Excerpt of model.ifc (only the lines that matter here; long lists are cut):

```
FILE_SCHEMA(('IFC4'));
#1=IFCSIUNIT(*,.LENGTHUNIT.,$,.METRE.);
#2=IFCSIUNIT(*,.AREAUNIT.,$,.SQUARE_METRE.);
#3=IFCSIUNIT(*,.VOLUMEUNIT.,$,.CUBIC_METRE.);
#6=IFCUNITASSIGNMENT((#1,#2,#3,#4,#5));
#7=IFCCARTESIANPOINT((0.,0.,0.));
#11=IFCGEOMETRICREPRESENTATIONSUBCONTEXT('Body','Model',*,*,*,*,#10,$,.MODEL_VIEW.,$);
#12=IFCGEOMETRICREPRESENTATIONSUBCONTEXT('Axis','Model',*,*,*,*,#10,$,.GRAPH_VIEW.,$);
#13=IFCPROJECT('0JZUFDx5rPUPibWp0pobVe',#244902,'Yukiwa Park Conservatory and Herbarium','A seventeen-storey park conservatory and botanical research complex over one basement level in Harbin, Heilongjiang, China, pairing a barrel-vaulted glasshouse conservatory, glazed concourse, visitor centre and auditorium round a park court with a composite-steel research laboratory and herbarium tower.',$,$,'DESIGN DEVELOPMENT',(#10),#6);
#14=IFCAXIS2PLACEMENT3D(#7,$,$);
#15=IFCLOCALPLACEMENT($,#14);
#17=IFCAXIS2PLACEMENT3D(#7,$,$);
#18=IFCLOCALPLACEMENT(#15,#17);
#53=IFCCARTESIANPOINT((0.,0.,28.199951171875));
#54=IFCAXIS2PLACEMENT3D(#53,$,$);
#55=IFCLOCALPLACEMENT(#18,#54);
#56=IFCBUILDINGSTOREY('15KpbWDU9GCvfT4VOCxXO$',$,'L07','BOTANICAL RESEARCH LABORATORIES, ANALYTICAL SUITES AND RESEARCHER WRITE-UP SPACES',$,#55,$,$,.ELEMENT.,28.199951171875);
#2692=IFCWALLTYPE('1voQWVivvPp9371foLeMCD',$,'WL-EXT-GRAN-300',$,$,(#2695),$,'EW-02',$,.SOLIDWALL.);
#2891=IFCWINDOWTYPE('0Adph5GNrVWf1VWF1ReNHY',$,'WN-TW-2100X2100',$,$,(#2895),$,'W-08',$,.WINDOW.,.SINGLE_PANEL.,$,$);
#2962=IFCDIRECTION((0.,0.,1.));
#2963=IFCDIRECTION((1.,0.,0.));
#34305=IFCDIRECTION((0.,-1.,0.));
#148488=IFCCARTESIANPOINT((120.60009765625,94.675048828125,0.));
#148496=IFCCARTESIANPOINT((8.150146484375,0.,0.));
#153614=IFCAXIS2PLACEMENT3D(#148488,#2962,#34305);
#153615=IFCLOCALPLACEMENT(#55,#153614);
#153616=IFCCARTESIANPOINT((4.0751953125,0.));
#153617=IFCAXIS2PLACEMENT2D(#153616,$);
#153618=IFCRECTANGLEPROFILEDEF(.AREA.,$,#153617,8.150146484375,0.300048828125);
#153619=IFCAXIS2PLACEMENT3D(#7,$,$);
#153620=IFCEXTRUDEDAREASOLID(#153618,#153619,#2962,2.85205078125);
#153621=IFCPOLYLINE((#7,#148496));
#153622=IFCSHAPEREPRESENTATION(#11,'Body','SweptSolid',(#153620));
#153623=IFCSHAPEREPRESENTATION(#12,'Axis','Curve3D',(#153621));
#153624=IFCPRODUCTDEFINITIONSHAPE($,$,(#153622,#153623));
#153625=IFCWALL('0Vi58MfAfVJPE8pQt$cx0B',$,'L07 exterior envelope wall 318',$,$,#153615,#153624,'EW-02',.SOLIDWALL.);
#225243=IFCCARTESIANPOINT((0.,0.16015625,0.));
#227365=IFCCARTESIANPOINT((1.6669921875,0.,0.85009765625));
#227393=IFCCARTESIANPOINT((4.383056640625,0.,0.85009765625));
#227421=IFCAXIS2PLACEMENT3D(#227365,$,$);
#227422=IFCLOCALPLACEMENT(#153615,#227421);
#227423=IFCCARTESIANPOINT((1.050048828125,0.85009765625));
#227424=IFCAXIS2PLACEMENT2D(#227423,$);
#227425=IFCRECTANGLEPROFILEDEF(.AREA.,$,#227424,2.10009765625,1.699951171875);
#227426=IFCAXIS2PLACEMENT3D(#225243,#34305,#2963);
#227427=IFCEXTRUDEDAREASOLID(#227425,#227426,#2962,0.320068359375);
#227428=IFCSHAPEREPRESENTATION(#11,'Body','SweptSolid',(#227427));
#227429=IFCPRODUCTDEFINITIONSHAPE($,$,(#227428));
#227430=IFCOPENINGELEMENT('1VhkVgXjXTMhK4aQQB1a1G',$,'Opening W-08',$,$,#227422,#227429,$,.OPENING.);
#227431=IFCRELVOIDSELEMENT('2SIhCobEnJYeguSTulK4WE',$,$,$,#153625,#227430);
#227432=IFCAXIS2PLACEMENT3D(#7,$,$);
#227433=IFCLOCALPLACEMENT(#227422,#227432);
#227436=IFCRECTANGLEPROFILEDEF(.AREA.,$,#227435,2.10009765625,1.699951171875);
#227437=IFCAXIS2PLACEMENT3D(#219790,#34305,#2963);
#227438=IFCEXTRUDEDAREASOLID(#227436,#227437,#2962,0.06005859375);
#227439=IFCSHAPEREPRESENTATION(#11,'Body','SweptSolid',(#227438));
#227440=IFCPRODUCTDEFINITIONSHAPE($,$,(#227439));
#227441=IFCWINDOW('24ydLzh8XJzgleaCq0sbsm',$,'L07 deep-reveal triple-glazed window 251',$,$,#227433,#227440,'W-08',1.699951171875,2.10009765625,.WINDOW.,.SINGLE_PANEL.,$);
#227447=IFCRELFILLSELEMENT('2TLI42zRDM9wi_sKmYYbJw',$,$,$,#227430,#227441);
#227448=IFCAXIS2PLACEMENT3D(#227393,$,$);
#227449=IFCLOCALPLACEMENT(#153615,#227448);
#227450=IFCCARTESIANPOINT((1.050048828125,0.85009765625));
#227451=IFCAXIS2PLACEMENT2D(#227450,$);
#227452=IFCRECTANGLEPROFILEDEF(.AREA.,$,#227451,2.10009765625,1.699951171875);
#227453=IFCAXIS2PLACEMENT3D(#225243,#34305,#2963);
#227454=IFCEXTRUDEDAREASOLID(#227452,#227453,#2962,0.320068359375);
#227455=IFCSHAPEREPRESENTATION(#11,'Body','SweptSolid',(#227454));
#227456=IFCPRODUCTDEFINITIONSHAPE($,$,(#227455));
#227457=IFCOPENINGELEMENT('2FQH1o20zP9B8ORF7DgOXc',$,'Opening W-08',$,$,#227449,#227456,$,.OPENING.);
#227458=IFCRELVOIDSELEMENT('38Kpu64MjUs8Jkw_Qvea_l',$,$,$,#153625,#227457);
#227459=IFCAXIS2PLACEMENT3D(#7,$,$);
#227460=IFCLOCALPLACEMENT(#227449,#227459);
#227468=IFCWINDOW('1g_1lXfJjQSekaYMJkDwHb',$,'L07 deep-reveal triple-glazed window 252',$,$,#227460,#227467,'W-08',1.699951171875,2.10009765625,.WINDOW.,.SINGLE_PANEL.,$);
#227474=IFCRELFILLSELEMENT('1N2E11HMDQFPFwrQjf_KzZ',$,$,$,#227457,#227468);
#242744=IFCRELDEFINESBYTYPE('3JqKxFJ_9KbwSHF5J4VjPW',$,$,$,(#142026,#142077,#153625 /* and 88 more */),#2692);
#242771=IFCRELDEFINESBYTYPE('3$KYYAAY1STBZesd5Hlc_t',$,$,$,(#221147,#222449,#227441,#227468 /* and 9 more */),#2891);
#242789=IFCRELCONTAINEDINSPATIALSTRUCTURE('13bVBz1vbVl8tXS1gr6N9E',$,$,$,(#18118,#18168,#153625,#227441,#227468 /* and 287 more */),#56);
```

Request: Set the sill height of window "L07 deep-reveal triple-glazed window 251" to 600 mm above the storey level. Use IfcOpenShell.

```python
import numpy as np
import ifcopenshell
import ifcopenshell.api.geometry
import ifcopenshell.geom
import ifcopenshell.util.element
import ifcopenshell.util.placement
import ifcopenshell.util.shape
import ifcopenshell.util.unit

model = ifcopenshell.open("model.ifc")
unit_scale = ifcopenshell.util.unit.calculate_unit_scale(model)

window = model.by_guid("24ydLzh8XJzgleaCq0sbsm")
opening = window.FillsVoids[0].RelatingOpeningElement
storey = ifcopenshell.util.element.get_container(window, ifc_class="IfcBuildingStorey")
level = ifcopenshell.util.placement.get_local_placement(storey.ObjectPlacement)[2, 3]

# The opening's origin need not be at the sill, so measure its lowest point.
shape = ifcopenshell.geom.create_shape(ifcopenshell.geom.settings(), opening)
bottom = ifcopenshell.util.shape.get_shape_bottom_elevation(shape, shape.geometry) / unit_scale
dz = level + 0.6 - bottom

shift = np.array([0.0, 0.0, dz])
# The window is placed relative to its opening, so it follows when the opening moves.
matrix = ifcopenshell.util.placement.get_local_placement(opening.ObjectPlacement)
matrix[:3, 3] += shift
ifcopenshell.api.geometry.edit_object_placement(
    model, product=opening, matrix=matrix, is_si=False, should_transform_children=True
)

print(f"moved by {dz * unit_scale:+.3f} m")

model.write("model_rev.ifc")
```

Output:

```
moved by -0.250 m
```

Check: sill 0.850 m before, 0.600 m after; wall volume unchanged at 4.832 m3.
